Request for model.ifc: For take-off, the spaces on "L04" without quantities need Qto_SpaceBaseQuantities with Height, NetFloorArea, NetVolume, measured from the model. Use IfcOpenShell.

First a look at what the model holds.

```python
import ifcopenshell
import ifcopenshell.util.element
import ifcopenshell.util.unit

model = ifcopenshell.open("model.ifc")
print(model.schema)
for unit_type in ("LENGTHUNIT", "AREAUNIT", "VOLUMEUNIT"):
    print(unit_type, ifcopenshell.util.unit.calculate_unit_scale(model, unit_type))
storey = next(s for s in model.by_type("IfcBuildingStorey") if s.Name == "L04")
spaces = [e for e in ifcopenshell.util.element.get_decomposition(storey) if e.is_a("IfcSpace")]
for e in sorted(spaces, key=lambda e: e.id()):
    print(e.id(), e.is_a(), e.Name, list(ifcopenshell.util.element.get_psets(e, qtos_only=True)), sep=" | ")
```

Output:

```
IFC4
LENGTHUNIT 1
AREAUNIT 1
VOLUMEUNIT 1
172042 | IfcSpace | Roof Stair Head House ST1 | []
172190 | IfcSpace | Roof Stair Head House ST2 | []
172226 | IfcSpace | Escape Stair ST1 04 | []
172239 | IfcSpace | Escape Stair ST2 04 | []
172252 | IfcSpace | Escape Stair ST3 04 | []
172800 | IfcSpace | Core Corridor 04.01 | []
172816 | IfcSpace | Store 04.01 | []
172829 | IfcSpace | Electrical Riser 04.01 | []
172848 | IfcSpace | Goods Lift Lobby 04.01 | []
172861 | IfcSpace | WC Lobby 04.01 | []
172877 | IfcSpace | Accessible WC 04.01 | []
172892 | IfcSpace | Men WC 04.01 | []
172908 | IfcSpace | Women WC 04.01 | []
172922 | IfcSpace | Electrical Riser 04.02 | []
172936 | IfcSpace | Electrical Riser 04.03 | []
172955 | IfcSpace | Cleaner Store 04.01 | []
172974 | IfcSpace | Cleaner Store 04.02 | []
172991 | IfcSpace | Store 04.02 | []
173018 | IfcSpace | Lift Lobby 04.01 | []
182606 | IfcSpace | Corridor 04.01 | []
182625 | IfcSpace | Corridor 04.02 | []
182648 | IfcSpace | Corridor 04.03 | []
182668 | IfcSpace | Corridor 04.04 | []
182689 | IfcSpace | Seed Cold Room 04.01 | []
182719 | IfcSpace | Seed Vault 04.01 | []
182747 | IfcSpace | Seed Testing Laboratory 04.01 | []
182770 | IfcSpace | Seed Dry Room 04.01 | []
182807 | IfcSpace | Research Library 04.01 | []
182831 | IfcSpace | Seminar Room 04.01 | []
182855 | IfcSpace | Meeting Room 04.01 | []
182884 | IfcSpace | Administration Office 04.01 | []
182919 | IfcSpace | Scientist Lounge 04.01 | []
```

```python
import ifcopenshell
import ifcopenshell.api.pset
import ifcopenshell.geom
import ifcopenshell.util.element
import ifcopenshell.util.shape
import ifcopenshell.util.unit

model = ifcopenshell.open("model.ifc")
unit_scale = ifcopenshell.util.unit.calculate_unit_scale(model)
area_scale = ifcopenshell.util.unit.calculate_unit_scale(model, "AREAUNIT")
volume_scale = ifcopenshell.util.unit.calculate_unit_scale(model, "VOLUMEUNIT")
settings = ifcopenshell.geom.settings()

storey = next(s for s in model.by_type("IfcBuildingStorey") if s.Name == "L04")
spaces = [e for e in ifcopenshell.util.element.get_decomposition(storey) if e.is_a("IfcSpace")]

for e in sorted(spaces, key=lambda e: e.id()):
    if ifcopenshell.util.element.get_psets(e, qtos_only=True, should_inherit=False):
        continue
    # Geometry comes back in metres, in the element's own axes.
    shape = ifcopenshell.geom.create_shape(settings, e)
    values = {
        "Height": ifcopenshell.util.shape.get_z(shape.geometry) / unit_scale,
        "NetFloorArea": ifcopenshell.util.shape.get_footprint_area(shape.geometry) / area_scale,
        "NetVolume": ifcopenshell.util.shape.get_volume(shape.geometry) / volume_scale,
    }
    qto = ifcopenshell.api.pset.add_qto(model, product=e, name="Qto_SpaceBaseQuantities")
    ifcopenshell.api.pset.edit_qto(model, qto=qto, properties=values)
    print(e.id(), {k: round(v, 3) for k, v in values.items()})

model.write("model_updated.ifc")
```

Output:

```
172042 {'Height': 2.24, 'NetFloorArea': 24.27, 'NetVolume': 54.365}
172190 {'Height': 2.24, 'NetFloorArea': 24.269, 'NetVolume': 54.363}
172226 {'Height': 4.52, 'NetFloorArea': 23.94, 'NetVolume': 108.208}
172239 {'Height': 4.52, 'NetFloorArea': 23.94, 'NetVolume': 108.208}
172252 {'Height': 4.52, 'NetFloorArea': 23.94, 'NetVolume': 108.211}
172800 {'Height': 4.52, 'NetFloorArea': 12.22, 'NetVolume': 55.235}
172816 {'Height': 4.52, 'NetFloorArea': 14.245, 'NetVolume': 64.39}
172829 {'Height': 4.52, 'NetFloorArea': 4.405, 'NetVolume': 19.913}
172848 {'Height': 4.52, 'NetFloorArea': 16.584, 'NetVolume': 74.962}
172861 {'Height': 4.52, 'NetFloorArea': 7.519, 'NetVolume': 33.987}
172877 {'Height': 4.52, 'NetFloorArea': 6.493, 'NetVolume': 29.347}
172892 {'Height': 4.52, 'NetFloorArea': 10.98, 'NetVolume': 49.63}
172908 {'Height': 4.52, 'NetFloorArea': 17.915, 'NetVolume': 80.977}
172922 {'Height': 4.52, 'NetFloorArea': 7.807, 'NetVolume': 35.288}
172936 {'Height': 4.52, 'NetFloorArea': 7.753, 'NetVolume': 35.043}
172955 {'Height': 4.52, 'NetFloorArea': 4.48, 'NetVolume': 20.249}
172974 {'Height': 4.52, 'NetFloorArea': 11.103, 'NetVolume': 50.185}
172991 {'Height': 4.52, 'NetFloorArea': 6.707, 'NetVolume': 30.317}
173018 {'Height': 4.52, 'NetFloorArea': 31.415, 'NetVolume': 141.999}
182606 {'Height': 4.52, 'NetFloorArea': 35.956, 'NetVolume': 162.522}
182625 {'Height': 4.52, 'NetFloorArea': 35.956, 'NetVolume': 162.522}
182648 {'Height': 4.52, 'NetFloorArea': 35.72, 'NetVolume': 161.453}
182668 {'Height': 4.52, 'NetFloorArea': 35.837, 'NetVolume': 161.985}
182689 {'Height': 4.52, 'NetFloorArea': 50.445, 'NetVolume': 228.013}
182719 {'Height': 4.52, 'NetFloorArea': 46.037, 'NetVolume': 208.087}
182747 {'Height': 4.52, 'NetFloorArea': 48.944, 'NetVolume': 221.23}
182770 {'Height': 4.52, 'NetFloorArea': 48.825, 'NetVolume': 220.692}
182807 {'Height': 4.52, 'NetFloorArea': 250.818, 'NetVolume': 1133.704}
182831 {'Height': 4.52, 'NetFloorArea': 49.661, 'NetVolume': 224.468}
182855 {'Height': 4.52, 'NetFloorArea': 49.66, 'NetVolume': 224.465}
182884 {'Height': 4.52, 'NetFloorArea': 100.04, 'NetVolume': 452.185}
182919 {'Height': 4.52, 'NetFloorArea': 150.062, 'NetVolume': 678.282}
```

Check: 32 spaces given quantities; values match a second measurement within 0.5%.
